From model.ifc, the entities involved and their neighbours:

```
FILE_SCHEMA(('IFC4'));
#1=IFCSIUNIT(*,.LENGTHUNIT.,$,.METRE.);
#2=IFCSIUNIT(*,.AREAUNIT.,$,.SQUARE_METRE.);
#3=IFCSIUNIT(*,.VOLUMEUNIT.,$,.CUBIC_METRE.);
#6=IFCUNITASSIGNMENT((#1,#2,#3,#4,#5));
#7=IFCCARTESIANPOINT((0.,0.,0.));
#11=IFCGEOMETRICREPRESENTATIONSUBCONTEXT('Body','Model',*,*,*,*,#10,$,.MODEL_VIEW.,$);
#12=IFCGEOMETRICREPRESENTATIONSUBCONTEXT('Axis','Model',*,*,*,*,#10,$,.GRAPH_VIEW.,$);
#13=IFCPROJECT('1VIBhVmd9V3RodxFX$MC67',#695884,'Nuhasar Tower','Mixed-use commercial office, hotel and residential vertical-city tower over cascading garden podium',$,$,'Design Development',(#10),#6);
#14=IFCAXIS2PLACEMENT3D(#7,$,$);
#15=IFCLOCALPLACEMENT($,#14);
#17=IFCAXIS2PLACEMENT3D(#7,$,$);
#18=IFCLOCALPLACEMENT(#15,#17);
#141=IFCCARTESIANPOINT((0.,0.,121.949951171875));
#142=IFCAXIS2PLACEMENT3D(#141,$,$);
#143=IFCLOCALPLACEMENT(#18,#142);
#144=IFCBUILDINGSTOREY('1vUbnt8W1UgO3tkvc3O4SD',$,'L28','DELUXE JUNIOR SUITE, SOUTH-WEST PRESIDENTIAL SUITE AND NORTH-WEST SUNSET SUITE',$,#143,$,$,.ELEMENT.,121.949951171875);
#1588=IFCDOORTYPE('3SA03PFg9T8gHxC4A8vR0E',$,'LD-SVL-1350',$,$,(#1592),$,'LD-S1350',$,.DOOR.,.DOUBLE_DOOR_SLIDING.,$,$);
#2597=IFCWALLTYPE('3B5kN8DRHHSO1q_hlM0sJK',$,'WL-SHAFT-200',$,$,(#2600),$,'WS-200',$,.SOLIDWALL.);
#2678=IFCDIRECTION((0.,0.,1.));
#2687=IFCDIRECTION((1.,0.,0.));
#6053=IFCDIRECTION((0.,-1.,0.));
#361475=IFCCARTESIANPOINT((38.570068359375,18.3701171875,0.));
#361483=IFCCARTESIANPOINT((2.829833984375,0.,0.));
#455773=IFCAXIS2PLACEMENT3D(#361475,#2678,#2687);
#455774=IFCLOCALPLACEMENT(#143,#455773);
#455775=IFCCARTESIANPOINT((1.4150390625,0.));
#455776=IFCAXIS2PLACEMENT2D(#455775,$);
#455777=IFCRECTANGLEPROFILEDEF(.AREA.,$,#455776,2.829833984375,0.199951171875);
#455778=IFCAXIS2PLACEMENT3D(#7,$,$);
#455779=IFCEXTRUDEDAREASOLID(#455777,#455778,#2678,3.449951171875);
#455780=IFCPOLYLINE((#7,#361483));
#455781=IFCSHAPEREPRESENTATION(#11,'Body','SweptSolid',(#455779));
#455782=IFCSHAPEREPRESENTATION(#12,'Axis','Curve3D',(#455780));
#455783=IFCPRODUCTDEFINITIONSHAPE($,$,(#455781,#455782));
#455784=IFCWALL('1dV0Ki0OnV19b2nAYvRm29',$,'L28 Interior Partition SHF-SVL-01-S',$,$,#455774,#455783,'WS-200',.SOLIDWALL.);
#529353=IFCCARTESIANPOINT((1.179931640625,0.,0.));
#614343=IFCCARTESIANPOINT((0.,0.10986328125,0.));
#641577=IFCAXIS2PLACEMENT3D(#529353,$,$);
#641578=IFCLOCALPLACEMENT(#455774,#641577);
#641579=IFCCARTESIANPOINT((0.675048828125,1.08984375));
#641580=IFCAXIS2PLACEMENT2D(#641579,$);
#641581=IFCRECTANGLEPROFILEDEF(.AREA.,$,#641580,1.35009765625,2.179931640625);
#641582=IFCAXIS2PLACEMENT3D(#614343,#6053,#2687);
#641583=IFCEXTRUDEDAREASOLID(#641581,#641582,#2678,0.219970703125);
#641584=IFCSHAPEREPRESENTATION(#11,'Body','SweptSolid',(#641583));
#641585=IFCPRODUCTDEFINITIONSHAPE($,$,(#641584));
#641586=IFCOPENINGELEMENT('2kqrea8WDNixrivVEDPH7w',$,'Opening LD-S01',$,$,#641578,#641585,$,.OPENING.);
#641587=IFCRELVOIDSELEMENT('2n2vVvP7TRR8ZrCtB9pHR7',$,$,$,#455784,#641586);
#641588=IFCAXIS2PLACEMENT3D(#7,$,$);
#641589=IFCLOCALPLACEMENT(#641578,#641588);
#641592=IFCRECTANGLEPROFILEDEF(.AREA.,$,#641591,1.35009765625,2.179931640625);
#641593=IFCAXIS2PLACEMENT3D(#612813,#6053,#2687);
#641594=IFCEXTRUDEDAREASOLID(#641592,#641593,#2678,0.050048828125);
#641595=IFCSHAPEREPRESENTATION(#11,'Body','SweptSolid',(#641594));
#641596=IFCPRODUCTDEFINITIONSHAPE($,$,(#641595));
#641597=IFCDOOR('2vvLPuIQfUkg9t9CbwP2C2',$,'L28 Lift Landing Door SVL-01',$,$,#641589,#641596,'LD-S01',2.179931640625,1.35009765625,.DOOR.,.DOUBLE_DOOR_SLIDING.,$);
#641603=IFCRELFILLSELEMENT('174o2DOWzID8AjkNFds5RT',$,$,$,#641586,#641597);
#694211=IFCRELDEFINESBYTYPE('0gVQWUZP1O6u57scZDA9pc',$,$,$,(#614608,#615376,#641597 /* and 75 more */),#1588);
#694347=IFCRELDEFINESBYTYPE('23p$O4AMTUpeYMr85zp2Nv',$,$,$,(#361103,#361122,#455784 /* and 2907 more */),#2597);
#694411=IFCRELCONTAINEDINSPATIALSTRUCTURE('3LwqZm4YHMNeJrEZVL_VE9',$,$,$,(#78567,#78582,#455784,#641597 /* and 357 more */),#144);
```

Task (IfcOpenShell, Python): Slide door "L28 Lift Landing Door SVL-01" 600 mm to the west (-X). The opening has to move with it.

```python
import ifcopenshell
import ifcopenshell.api.geometry
import ifcopenshell.util.placement

model = ifcopenshell.open("model.ifc")

door = model.by_id(641597)
opening = door.FillsVoids[0].RelatingOpeningElement
wall = opening.VoidsElements[0].RelatingBuildingElement

wall_matrix = ifcopenshell.util.placement.get_local_placement(wall.ObjectPlacement)
shift = wall_matrix[:3, 0] * -0.6
before = ifcopenshell.util.placement.get_local_placement(door.ObjectPlacement)[:3, 3].copy()

# The door is placed relative to its opening, so it follows when the opening moves.
matrix = ifcopenshell.util.placement.get_local_placement(opening.ObjectPlacement)
matrix[:3, 3] += shift
ifcopenshell.api.geometry.edit_object_placement(
    model, product=opening, matrix=matrix, is_si=False, should_transform_children=True
)

after = ifcopenshell.util.placement.get_local_placement(door.ObjectPlacement)[:3, 3]
print("door moved by", (after - before).round(3) + 0.0)

model.write("model_updated.ifc")
```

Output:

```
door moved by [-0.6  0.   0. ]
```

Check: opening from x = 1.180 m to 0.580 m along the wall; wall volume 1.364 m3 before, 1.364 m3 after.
